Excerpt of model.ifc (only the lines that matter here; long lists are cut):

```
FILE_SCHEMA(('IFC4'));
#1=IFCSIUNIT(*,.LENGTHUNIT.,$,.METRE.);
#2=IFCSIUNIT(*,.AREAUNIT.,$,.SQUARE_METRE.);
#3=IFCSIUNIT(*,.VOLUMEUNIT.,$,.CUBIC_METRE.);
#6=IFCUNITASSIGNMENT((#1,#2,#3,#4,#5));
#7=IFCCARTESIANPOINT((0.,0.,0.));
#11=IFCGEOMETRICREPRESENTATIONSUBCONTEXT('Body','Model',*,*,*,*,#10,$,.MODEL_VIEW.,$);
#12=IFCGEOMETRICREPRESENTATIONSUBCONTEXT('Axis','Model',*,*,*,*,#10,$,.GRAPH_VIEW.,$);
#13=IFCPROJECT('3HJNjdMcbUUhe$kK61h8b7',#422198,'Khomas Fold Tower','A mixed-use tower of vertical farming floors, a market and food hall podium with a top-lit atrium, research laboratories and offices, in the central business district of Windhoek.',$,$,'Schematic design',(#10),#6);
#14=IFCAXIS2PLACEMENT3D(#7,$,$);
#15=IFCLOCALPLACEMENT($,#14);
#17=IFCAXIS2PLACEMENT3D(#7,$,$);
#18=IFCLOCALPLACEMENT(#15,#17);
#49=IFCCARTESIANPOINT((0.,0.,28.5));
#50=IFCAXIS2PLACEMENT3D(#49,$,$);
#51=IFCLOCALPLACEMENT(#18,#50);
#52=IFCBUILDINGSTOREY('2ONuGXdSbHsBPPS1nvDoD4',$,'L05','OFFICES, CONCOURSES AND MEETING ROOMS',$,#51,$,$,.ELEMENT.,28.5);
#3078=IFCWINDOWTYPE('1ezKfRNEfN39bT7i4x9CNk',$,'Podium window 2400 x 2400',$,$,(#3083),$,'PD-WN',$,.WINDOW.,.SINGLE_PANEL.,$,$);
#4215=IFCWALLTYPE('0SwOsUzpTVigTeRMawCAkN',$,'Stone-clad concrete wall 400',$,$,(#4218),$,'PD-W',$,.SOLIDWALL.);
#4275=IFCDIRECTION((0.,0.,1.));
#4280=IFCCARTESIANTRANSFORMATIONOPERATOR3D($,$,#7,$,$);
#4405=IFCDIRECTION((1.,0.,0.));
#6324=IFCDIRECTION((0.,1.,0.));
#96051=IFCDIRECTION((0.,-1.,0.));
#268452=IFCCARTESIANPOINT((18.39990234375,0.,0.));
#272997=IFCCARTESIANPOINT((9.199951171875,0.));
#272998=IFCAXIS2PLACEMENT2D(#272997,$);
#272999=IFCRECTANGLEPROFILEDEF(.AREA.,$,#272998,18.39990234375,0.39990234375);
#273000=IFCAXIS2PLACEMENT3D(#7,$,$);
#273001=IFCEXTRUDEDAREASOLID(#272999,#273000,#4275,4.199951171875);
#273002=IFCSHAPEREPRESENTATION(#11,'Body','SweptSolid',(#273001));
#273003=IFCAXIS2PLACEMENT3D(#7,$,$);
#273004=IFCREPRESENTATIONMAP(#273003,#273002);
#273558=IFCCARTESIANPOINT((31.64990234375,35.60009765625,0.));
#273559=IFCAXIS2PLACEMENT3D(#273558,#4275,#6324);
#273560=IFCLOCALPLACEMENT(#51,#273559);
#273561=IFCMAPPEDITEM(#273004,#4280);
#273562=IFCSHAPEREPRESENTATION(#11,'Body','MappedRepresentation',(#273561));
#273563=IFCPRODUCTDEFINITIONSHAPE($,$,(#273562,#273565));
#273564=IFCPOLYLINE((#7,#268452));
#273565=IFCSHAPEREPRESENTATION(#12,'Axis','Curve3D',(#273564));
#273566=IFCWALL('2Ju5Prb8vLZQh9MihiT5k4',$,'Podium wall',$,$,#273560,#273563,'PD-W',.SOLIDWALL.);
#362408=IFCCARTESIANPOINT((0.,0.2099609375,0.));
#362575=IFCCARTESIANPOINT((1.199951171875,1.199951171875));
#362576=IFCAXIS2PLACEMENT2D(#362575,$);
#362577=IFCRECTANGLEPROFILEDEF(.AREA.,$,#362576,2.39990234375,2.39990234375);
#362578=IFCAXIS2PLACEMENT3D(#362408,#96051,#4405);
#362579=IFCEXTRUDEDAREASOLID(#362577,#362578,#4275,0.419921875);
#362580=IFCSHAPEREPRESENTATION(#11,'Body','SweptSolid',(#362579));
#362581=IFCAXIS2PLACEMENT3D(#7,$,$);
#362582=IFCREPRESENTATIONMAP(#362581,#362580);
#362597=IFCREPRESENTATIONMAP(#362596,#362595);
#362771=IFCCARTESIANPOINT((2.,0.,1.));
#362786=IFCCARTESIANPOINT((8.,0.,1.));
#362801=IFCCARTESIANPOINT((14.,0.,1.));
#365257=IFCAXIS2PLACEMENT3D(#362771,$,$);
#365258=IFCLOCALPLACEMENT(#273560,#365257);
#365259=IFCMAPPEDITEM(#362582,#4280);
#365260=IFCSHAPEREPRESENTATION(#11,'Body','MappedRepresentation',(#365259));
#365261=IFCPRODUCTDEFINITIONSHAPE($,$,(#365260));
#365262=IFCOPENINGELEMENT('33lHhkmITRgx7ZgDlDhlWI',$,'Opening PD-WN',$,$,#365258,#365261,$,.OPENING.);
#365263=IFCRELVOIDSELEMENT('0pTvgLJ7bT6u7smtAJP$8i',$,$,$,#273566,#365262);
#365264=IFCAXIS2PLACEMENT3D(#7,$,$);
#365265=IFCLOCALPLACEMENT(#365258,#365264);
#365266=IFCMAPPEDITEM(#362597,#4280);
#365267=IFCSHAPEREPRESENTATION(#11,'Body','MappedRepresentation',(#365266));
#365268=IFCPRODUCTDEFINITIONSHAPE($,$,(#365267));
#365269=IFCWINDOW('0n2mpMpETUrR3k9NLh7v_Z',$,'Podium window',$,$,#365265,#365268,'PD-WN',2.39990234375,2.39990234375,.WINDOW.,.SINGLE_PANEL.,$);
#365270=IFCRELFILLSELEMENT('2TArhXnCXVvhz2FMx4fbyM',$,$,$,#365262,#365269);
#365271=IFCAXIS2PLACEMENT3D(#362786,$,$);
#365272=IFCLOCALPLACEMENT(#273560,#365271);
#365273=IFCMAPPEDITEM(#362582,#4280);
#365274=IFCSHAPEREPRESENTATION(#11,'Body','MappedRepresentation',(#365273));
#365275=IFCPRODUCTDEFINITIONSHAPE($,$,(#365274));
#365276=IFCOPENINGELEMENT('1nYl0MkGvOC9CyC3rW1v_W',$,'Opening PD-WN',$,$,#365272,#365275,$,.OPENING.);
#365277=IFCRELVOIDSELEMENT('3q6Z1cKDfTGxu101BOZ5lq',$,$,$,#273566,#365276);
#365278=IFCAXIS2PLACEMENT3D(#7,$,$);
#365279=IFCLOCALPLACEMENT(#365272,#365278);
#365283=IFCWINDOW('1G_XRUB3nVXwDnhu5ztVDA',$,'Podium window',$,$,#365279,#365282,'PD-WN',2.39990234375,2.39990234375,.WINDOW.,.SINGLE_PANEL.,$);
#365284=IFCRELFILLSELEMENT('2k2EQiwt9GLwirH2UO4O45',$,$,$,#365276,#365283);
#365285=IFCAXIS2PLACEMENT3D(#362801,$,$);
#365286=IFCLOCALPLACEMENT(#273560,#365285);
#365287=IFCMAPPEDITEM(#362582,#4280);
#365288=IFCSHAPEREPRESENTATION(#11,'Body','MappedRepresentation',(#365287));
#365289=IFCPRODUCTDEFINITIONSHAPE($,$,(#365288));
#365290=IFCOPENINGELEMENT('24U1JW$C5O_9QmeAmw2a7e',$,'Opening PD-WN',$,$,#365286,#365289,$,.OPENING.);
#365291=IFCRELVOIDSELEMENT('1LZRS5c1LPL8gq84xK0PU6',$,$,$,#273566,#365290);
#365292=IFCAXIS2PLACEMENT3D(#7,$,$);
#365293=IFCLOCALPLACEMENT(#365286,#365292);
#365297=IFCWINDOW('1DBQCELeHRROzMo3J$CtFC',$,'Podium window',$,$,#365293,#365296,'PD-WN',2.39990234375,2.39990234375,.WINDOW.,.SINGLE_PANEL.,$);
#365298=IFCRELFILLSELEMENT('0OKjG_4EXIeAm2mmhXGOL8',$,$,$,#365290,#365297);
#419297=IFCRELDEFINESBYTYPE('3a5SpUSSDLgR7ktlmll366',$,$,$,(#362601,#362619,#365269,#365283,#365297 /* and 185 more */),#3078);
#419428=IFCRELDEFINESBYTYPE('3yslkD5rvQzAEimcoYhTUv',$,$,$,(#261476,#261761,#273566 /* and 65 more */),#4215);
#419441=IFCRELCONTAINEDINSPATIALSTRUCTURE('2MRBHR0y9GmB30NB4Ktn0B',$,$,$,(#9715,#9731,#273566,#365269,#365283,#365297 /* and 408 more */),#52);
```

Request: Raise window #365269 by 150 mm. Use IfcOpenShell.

```python
import numpy as np
import ifcopenshell
import ifcopenshell.api.geometry
import ifcopenshell.util.placement
import ifcopenshell.util.unit

model = ifcopenshell.open("model.ifc")
unit_scale = ifcopenshell.util.unit.calculate_unit_scale(model)

window = model.by_guid("0n2mpMpETUrR3k9NLh7v_Z")
opening = window.FillsVoids[0].RelatingOpeningElement
dz = 0.15 / unit_scale

shift = np.array([0.0, 0.0, dz])
# The window is placed relative to its opening, so it follows when the opening moves.
matrix = ifcopenshell.util.placement.get_local_placement(opening.ObjectPlacement)
matrix[:3, 3] += shift
ifcopenshell.api.geometry.edit_object_placement(
    model, product=opening, matrix=matrix, is_si=False, should_transform_children=True
)

print(f"moved by {dz * unit_scale:+.3f} m")

model.write("model_v2.ifc")
```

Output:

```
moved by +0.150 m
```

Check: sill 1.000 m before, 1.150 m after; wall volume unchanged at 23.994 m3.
